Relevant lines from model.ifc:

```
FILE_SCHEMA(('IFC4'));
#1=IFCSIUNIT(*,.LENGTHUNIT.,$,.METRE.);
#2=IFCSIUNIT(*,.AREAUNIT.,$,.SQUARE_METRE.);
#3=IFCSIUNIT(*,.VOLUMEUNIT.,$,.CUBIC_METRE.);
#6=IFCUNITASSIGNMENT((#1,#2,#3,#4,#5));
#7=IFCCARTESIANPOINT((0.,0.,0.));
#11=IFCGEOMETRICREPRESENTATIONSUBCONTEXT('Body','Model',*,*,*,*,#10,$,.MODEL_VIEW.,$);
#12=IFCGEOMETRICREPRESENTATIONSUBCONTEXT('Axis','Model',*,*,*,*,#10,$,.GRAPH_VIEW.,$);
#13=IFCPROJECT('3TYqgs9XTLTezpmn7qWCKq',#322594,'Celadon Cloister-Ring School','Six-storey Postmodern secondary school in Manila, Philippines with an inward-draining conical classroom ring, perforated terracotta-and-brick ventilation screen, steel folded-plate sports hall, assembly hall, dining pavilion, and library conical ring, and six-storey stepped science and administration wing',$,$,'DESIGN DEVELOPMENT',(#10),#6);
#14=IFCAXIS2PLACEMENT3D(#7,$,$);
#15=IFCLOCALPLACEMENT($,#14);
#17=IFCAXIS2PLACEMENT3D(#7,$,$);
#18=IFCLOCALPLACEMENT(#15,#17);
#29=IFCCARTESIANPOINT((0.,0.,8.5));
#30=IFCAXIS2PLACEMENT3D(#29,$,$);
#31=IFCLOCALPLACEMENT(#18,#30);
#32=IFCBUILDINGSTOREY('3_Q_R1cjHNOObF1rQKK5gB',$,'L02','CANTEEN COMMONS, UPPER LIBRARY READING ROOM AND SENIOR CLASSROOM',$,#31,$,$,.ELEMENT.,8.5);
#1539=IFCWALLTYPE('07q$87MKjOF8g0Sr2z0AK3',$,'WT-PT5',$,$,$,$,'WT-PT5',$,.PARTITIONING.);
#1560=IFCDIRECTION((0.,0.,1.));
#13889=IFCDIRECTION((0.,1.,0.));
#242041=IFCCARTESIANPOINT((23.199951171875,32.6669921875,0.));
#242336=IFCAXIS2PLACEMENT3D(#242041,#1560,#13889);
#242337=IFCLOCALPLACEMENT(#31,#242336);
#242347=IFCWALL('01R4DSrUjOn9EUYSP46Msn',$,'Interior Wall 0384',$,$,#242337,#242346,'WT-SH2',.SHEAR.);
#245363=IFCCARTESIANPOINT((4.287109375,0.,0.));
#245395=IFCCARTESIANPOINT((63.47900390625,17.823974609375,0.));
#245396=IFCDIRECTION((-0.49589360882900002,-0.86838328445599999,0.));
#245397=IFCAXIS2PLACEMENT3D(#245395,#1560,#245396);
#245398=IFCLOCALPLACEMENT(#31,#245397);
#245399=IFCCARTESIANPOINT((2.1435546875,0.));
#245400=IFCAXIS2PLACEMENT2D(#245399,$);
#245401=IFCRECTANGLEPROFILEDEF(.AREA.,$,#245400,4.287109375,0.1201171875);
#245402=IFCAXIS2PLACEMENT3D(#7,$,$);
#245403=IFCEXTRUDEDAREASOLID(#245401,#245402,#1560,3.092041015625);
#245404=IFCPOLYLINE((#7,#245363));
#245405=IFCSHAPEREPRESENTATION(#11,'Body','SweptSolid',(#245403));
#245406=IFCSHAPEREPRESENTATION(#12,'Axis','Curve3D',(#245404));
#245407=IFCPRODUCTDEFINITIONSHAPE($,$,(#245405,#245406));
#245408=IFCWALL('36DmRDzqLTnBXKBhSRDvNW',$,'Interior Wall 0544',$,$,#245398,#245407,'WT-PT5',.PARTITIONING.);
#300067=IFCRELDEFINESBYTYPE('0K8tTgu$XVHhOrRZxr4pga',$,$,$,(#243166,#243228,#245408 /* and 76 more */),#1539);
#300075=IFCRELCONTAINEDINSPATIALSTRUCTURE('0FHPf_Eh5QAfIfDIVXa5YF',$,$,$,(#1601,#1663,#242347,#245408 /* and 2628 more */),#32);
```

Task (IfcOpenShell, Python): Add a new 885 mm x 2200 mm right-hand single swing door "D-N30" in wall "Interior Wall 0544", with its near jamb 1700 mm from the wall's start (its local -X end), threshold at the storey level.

```python
import numpy as np
import ifcopenshell
import ifcopenshell.api.feature
import ifcopenshell.api.geometry
import ifcopenshell.api.root
import ifcopenshell.api.spatial
import ifcopenshell.geom
import ifcopenshell.util.element
import ifcopenshell.util.placement
import ifcopenshell.util.representation
import ifcopenshell.util.shape
import ifcopenshell.util.unit

model = ifcopenshell.open("model.ifc")
unit_scale = ifcopenshell.util.unit.calculate_unit_scale(model)
settings = ifcopenshell.geom.settings()


def volume(element):
    """Net volume in cubic metres, openings subtracted."""
    shape = ifcopenshell.geom.create_shape(settings, element)
    return ifcopenshell.util.shape.get_volume(shape.geometry)


wall = model.by_guid("36DmRDzqLTnBXKBhSRDvNW")
storey = ifcopenshell.util.element.get_container(wall, ifc_class="IfcBuildingStorey")
context = ifcopenshell.util.representation.get_context(model, "Model", "Body", "MODEL_VIEW")
before = volume(wall)

width, height, from_end, sill = 0.885, 2.2, 1.7, 0.0  # metres

# The wall runs along its own X axis, and the end named is its -X end.
wall_shape = ifcopenshell.geom.create_shape(settings, wall)
x, y, z = ifcopenshell.util.shape.get_vertices(wall_shape.geometry).T
start = x.min() + from_end
face, thickness = float(y.min()), float(y.max() - y.min())
wall_matrix = ifcopenshell.util.placement.get_local_placement(wall.ObjectPlacement)
level = ifcopenshell.util.placement.get_local_placement(storey.ObjectPlacement)[2, 3]


def in_wall(x, y):
    """Placement at x, y metres in the wall's axes, at sill height."""
    matrix = wall_matrix.copy()
    matrix[:, 3] = wall_matrix @ np.array([x / unit_scale, y / unit_scale, 0.0, 1.0])
    matrix[2, 3] = level + sill / unit_scale
    return matrix


# Opening: a box that overshoots both wall faces by 50 mm.
opening = ifcopenshell.api.root.create_entity(model, ifc_class="IfcOpeningElement", predefined_type="OPENING")
box = ifcopenshell.api.geometry.add_wall_representation(
    model, context=context, length=width, height=height, thickness=thickness + 0.1
)
ifcopenshell.api.geometry.assign_representation(model, product=opening, representation=box)
ifcopenshell.api.geometry.edit_object_placement(model, product=opening, matrix=in_wall(start, face - 0.05), is_si=False)
ifcopenshell.api.feature.add_feature(model, feature=opening, element=wall)

door = ifcopenshell.api.root.create_entity(model, ifc_class="IfcDoor", name="D-N30", predefined_type="DOOR")
door.OverallWidth, door.OverallHeight = width / unit_scale, height / unit_scale
door.OperationType = "SINGLE_SWING_RIGHT"
body = ifcopenshell.api.geometry.add_door_representation(
    model,
    context=context,
    overall_width=door.OverallWidth,
    overall_height=door.OverallHeight,
    operation_type="SINGLE_SWING_RIGHT",
    lining_properties={"LiningDepth": thickness / unit_scale, "ThresholdDepth": thickness / unit_scale},
)
ifcopenshell.api.geometry.assign_representation(model, product=door, representation=body)
ifcopenshell.api.spatial.assign_container(model, products=[door], relating_structure=storey)
ifcopenshell.api.feature.add_filling(model, opening=opening, element=door)

# The lining spans the wall, so the door starts at the wall face.
ifcopenshell.api.geometry.edit_object_placement(model, product=door, matrix=in_wall(start, face), is_si=False)

after = volume(wall)

print(f"wall volume {before:.3f} -> {after:.3f} m3")

model.write("model-out.ifc")
```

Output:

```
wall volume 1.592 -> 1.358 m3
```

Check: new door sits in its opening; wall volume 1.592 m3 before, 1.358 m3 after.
